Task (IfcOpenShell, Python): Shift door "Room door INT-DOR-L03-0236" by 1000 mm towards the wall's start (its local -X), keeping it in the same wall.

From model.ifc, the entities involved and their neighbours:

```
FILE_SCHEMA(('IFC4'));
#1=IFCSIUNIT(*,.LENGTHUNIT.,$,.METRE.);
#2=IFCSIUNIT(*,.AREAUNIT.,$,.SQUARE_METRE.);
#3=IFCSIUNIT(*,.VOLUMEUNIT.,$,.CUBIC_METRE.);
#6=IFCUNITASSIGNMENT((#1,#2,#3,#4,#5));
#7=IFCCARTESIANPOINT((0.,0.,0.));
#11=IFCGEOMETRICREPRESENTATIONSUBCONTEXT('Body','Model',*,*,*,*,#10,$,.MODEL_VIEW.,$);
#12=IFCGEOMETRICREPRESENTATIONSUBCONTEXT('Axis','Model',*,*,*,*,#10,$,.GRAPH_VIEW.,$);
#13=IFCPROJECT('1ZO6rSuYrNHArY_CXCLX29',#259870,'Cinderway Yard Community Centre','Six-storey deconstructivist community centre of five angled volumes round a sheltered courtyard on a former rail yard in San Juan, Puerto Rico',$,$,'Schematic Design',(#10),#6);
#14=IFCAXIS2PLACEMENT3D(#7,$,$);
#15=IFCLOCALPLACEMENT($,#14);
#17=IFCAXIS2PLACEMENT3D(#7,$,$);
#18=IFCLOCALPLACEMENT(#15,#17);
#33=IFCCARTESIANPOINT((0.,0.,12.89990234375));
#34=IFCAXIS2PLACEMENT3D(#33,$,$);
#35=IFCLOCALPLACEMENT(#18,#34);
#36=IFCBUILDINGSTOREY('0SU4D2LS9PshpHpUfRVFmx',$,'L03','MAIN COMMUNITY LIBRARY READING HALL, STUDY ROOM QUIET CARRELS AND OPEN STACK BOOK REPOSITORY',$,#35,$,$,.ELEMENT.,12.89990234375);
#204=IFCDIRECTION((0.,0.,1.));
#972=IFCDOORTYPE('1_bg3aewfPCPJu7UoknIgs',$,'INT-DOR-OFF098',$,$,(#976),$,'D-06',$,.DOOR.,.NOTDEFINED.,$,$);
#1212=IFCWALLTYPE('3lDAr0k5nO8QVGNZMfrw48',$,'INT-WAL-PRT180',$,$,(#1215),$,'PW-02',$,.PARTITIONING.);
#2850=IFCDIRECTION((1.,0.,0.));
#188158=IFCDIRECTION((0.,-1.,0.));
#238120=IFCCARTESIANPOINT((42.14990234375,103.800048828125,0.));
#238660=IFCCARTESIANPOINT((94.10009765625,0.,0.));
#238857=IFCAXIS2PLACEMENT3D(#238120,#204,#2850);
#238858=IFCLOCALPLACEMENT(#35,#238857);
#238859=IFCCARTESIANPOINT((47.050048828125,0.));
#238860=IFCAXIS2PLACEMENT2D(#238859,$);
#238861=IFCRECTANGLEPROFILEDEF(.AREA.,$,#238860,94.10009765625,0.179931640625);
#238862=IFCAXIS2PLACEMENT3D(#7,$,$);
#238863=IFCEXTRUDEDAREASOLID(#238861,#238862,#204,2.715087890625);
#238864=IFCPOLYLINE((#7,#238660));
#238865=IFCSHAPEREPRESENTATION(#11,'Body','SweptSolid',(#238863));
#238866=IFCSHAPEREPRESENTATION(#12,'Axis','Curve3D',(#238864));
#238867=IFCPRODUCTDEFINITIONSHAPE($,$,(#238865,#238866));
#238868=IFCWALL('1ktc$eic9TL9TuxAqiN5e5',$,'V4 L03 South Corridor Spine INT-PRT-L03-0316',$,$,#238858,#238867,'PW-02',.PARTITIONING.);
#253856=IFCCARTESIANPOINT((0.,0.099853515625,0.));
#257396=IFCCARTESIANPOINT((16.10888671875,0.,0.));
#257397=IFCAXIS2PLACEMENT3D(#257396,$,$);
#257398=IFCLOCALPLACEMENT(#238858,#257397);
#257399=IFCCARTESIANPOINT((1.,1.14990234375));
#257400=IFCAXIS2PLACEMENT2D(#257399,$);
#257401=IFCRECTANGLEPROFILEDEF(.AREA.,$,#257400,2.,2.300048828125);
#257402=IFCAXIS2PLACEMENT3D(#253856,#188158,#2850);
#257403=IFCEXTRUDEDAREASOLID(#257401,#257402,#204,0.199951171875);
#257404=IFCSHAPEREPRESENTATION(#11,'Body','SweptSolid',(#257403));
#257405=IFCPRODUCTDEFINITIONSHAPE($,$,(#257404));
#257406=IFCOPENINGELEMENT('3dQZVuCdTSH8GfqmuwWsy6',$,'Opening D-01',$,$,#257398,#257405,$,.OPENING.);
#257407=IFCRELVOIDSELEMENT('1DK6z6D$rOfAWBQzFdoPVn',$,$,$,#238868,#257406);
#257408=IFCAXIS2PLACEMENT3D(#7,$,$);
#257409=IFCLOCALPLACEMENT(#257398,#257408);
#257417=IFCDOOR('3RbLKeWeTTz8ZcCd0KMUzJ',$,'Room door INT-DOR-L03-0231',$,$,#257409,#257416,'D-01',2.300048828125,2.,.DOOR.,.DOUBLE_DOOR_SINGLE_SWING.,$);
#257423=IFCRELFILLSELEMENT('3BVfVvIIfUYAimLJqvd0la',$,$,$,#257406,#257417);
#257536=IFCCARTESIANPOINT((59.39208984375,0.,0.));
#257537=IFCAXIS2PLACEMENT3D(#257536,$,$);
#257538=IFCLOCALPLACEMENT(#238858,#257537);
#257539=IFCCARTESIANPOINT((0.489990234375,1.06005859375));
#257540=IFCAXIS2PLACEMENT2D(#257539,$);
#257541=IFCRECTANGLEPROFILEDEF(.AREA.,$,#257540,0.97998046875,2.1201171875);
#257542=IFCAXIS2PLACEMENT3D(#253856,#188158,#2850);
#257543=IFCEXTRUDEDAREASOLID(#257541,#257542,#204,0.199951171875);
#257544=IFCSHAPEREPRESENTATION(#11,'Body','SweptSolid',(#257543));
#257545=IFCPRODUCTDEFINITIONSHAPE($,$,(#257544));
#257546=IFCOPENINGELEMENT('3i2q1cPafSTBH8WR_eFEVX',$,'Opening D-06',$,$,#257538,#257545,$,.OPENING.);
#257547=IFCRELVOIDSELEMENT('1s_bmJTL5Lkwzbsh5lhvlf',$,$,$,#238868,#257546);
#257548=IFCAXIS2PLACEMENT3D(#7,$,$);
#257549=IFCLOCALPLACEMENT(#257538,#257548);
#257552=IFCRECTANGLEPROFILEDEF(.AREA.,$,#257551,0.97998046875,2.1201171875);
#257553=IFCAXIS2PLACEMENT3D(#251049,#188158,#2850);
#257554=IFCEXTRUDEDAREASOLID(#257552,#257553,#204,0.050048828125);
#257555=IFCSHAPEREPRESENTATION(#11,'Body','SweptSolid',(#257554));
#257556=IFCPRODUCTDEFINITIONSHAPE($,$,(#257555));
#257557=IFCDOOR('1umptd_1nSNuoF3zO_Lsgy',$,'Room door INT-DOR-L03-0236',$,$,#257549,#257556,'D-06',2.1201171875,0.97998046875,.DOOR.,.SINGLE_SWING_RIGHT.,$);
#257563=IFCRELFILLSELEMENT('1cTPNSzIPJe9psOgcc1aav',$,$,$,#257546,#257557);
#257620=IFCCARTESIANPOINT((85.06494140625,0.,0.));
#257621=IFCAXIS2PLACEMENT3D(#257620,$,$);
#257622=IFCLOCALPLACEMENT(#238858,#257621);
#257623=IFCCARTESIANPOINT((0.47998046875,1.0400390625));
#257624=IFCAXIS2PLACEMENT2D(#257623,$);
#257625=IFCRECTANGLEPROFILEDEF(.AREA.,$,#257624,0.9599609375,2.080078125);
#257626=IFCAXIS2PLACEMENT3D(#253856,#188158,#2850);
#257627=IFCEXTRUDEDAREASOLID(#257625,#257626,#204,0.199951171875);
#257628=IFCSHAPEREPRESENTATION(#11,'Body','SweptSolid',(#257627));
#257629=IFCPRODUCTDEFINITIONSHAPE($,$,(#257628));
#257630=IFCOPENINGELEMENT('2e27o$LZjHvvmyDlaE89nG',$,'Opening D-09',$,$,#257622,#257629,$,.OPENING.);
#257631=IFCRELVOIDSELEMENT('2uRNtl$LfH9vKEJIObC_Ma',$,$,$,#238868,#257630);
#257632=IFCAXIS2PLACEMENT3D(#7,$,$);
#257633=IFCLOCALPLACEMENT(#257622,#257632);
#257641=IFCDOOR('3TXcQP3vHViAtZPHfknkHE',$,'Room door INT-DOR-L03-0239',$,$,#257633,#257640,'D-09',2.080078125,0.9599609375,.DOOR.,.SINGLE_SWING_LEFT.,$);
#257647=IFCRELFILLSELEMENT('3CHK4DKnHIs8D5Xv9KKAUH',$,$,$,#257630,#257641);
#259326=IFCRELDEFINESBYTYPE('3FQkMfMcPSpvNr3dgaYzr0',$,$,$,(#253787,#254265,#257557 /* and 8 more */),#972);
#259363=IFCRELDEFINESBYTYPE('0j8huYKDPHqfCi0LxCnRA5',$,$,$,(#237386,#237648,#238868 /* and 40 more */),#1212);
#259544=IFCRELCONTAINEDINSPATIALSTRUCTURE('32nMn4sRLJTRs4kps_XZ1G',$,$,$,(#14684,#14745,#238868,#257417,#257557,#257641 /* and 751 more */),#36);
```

```python
import ifcopenshell
import ifcopenshell.api.geometry
import ifcopenshell.util.placement
import ifcopenshell.util.unit

model = ifcopenshell.open("model.ifc")
unit_scale = ifcopenshell.util.unit.calculate_unit_scale(model)

door = model.by_guid("1umptd_1nSNuoF3zO_Lsgy")
opening = door.FillsVoids[0].RelatingOpeningElement
wall = opening.VoidsElements[0].RelatingBuildingElement

wall_matrix = ifcopenshell.util.placement.get_local_placement(wall.ObjectPlacement)
shift = wall_matrix[:3, 0] * -1 / unit_scale
before = ifcopenshell.util.placement.get_local_placement(door.ObjectPlacement)[:3, 3].copy()

# The door is placed relative to its opening, so it follows when the opening moves.
matrix = ifcopenshell.util.placement.get_local_placement(opening.ObjectPlacement)
matrix[:3, 3] += shift
ifcopenshell.api.geometry.edit_object_placement(
    model, product=opening, matrix=matrix, is_si=False, should_transform_children=True
)

after = ifcopenshell.util.placement.get_local_placement(door.ObjectPlacement)[:3, 3]
print("door moved by", (after - before).round(3) + 0.0)

model.write("model_edited.ifc")
```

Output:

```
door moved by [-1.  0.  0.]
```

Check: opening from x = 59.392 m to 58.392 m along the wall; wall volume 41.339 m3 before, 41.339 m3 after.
